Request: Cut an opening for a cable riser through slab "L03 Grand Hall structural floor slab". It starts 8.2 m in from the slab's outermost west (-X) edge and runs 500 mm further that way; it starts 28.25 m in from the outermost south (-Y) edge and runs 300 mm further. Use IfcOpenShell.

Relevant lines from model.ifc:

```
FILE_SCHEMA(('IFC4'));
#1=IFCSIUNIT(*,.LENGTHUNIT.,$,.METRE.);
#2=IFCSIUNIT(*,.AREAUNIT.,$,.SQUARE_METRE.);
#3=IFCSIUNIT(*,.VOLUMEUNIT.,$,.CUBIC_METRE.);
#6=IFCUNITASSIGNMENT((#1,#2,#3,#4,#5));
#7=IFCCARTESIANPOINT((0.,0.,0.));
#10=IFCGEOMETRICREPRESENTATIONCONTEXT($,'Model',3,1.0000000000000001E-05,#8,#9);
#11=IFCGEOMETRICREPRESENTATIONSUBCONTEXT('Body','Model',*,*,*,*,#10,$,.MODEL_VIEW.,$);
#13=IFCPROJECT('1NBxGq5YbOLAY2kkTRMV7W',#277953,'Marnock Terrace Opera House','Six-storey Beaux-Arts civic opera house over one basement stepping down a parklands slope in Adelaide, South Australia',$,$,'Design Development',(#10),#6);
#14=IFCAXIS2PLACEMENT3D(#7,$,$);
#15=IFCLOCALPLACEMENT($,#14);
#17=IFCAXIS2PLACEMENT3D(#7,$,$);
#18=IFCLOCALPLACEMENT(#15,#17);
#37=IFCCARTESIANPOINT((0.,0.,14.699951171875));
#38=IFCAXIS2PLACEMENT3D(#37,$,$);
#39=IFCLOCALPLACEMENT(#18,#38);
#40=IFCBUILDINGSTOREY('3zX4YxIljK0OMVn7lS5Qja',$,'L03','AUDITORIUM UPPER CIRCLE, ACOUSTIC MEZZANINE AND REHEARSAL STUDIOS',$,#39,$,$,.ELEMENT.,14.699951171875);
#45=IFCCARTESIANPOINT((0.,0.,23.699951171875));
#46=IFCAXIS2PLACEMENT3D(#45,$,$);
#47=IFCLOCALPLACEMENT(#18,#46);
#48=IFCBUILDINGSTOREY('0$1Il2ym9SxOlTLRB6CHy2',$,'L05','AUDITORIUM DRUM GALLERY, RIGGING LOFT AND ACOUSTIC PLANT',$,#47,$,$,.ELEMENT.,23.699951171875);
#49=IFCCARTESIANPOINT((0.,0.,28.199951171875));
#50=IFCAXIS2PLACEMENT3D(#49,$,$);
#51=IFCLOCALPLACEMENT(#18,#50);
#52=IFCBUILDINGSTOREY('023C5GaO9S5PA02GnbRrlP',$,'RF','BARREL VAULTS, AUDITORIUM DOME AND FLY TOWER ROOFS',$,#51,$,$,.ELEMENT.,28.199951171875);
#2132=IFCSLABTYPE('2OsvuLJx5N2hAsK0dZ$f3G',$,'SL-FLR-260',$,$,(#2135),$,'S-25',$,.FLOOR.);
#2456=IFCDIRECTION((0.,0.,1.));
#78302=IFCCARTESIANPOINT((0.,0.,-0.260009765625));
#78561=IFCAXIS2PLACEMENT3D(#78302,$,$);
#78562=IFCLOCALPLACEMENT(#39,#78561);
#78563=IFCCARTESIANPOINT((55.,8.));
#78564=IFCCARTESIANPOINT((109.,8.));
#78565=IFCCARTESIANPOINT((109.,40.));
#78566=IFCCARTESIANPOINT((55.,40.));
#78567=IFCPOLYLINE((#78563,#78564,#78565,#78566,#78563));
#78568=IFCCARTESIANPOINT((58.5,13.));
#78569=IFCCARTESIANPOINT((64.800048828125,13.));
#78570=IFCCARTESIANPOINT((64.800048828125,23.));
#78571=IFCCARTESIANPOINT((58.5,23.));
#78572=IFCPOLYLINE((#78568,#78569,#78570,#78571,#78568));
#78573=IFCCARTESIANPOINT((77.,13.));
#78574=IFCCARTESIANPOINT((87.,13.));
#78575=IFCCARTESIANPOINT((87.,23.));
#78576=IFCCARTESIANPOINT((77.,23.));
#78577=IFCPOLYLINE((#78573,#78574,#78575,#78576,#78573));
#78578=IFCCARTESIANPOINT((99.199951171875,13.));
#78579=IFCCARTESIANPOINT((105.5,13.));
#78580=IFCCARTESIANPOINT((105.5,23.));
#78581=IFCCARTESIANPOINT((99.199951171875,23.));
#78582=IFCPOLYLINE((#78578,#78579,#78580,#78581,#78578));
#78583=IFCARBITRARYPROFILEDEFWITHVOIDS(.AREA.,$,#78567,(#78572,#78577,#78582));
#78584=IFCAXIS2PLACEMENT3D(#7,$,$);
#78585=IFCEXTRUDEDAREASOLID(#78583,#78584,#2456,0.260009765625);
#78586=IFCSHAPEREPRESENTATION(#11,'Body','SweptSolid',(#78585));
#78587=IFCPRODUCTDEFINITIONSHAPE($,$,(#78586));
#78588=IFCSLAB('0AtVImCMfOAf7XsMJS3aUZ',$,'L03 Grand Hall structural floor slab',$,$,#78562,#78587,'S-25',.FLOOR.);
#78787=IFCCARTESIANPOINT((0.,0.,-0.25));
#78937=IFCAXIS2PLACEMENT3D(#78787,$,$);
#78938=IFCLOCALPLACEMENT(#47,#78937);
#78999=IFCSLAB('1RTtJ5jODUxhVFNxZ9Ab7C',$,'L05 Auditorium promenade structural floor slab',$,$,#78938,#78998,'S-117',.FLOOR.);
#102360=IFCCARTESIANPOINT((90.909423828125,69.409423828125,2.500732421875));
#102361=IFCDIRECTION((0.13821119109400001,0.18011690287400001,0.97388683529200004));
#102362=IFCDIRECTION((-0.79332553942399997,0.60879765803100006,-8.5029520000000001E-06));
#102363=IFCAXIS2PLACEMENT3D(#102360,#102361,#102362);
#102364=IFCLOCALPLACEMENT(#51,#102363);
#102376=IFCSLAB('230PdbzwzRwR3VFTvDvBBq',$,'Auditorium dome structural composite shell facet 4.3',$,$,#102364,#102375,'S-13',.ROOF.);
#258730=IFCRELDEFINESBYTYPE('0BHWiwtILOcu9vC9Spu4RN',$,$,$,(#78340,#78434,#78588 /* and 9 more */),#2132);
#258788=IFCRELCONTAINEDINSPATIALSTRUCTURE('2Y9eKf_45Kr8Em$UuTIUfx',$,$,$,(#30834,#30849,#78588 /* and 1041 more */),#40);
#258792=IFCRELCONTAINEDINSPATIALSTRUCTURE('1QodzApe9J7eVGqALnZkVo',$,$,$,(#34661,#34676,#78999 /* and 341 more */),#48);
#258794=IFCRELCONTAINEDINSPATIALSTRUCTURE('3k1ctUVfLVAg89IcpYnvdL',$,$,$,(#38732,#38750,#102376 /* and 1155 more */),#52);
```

```python
import numpy as np
import ifcopenshell
import ifcopenshell.api.feature
import ifcopenshell.api.geometry
import ifcopenshell.api.root
import ifcopenshell.geom
import ifcopenshell.util.placement
import ifcopenshell.util.representation
import ifcopenshell.util.shape
import ifcopenshell.util.unit

model = ifcopenshell.open("model.ifc")
unit_scale = ifcopenshell.util.unit.calculate_unit_scale(model)
settings = ifcopenshell.geom.settings()


def volume(element):
    """Net volume in cubic metres, openings subtracted."""
    shape = ifcopenshell.geom.create_shape(settings, element)
    return ifcopenshell.util.shape.get_volume(shape.geometry)


slab = model.by_id(78588)
before = volume(slab)

# Extent in the slab's own axes, in metres. The edges named are its -X and -Y sides.
slab_shape = ifcopenshell.geom.create_shape(settings, slab)
vertices = ifcopenshell.util.shape.get_vertices(slab_shape.geometry)
x_min, y_min, bottom = vertices.min(axis=0)
top = vertices[:, 2].max()

opening = ifcopenshell.api.root.create_entity(model, ifc_class="IfcOpeningElement", name="Cable riser opening", predefined_type="OPENING")
context = ifcopenshell.util.representation.get_context(model, "Model", "Body", "MODEL_VIEW")
width, depth = 0.5, 0.3
outline = [(0.0, 0.0), (width, 0.0), (width, depth), (0.0, depth), (0.0, 0.0)]
# Overshoot both faces by 50 mm so the cut is clean.
shape = ifcopenshell.api.geometry.add_slab_representation(
    model, context=context, depth=top - bottom + 0.1, polyline=outline
)
ifcopenshell.api.geometry.assign_representation(model, product=opening, representation=shape)

matrix = ifcopenshell.util.placement.get_local_placement(slab.ObjectPlacement)
matrix[:, 3] = matrix @ np.append(np.array([x_min + 8.2, y_min + 28.25, bottom - 0.05]) / unit_scale, 1.0)
ifcopenshell.api.geometry.edit_object_placement(model, product=opening, matrix=matrix, is_si=False)
ifcopenshell.api.feature.add_feature(model, feature=opening, element=slab)

after = volume(slab)

print(f"slab volume {before:.3f} -> {after:.3f} m3")

model.write("model_edited.ifc")
```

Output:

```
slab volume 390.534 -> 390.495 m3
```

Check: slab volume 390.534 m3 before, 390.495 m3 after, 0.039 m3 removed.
